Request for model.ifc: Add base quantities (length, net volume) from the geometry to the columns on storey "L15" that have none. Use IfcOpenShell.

First a look at what the model holds.

```python
import ifcopenshell
import ifcopenshell.util.element
import ifcopenshell.util.unit

model = ifcopenshell.open("model.ifc")
print(model.schema)
for unit_type in ("LENGTHUNIT", "AREAUNIT", "VOLUMEUNIT"):
    print(unit_type, ifcopenshell.util.unit.calculate_unit_scale(model, unit_type))
storey = next(s for s in model.by_type("IfcBuildingStorey") if s.Name == "L15")
columns = [e for e in ifcopenshell.util.element.get_decomposition(storey) if e.is_a("IfcColumn")]
for e in sorted(columns, key=lambda e: e.id()):
    print(e.id(), e.is_a(), e.Name, list(ifcopenshell.util.element.get_psets(e, qtos_only=True)), sep=" | ")
```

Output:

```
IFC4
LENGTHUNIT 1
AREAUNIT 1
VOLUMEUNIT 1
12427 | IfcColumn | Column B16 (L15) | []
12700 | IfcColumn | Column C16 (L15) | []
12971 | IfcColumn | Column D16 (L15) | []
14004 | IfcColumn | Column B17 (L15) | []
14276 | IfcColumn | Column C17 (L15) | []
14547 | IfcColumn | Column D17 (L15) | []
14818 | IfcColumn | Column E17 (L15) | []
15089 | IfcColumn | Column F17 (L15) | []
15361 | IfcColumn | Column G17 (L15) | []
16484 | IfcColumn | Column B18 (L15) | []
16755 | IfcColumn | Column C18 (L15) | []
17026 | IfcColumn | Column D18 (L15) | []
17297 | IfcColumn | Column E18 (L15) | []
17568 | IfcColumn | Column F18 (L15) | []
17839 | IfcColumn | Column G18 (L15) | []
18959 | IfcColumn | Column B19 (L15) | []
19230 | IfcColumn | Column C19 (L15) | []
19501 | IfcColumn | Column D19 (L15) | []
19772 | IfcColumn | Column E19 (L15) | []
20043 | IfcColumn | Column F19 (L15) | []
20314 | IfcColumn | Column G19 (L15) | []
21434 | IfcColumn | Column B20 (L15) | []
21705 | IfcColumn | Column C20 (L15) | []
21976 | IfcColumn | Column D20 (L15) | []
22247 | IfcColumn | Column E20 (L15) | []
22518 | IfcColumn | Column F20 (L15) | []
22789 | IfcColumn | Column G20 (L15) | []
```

```python
import ifcopenshell
import ifcopenshell.api.pset
import ifcopenshell.geom
import ifcopenshell.util.element
import ifcopenshell.util.shape
import ifcopenshell.util.unit

model = ifcopenshell.open("model.ifc")
unit_scale = ifcopenshell.util.unit.calculate_unit_scale(model)
volume_scale = ifcopenshell.util.unit.calculate_unit_scale(model, "VOLUMEUNIT")
settings = ifcopenshell.geom.settings()

storey = next(s for s in model.by_type("IfcBuildingStorey") if s.Name == "L15")
columns = [e for e in ifcopenshell.util.element.get_decomposition(storey) if e.is_a("IfcColumn")]

for e in sorted(columns, key=lambda e: e.id()):
    if ifcopenshell.util.element.get_psets(e, qtos_only=True, should_inherit=False):
        continue
    # Geometry comes back in metres, in the element's own axes.
    shape = ifcopenshell.geom.create_shape(settings, e)
    values = {
        "Length": ifcopenshell.util.shape.get_z(shape.geometry) / unit_scale,
        "NetVolume": ifcopenshell.util.shape.get_volume(shape.geometry) / volume_scale,
    }
    qto = ifcopenshell.api.pset.add_qto(model, product=e, name="Qto_ColumnBaseQuantities")
    ifcopenshell.api.pset.edit_qto(model, qto=qto, properties=values)
    print(e.id(), {k: round(v, 3) for k, v in values.items()})

model.write("model_rev.ifc")
```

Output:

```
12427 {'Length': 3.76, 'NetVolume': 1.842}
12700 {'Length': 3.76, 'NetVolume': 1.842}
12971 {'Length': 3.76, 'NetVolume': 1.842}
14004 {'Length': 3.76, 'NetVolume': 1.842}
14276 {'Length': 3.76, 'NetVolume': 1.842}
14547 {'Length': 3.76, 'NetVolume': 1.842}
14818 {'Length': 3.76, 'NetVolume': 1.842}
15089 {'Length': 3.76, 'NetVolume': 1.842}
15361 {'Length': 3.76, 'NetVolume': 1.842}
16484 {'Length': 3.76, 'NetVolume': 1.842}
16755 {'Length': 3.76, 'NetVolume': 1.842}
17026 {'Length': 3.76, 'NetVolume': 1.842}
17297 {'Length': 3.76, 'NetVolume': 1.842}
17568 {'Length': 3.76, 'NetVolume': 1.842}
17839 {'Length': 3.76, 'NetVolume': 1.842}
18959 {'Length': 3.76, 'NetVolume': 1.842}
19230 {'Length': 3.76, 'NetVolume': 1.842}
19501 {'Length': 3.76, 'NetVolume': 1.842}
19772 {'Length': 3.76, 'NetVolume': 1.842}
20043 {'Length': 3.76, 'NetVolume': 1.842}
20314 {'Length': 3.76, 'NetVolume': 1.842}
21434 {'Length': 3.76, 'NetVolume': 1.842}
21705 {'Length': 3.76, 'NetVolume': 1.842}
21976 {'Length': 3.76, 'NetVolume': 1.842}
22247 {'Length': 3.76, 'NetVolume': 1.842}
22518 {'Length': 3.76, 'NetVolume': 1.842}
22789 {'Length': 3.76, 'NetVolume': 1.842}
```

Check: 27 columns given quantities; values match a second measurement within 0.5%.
